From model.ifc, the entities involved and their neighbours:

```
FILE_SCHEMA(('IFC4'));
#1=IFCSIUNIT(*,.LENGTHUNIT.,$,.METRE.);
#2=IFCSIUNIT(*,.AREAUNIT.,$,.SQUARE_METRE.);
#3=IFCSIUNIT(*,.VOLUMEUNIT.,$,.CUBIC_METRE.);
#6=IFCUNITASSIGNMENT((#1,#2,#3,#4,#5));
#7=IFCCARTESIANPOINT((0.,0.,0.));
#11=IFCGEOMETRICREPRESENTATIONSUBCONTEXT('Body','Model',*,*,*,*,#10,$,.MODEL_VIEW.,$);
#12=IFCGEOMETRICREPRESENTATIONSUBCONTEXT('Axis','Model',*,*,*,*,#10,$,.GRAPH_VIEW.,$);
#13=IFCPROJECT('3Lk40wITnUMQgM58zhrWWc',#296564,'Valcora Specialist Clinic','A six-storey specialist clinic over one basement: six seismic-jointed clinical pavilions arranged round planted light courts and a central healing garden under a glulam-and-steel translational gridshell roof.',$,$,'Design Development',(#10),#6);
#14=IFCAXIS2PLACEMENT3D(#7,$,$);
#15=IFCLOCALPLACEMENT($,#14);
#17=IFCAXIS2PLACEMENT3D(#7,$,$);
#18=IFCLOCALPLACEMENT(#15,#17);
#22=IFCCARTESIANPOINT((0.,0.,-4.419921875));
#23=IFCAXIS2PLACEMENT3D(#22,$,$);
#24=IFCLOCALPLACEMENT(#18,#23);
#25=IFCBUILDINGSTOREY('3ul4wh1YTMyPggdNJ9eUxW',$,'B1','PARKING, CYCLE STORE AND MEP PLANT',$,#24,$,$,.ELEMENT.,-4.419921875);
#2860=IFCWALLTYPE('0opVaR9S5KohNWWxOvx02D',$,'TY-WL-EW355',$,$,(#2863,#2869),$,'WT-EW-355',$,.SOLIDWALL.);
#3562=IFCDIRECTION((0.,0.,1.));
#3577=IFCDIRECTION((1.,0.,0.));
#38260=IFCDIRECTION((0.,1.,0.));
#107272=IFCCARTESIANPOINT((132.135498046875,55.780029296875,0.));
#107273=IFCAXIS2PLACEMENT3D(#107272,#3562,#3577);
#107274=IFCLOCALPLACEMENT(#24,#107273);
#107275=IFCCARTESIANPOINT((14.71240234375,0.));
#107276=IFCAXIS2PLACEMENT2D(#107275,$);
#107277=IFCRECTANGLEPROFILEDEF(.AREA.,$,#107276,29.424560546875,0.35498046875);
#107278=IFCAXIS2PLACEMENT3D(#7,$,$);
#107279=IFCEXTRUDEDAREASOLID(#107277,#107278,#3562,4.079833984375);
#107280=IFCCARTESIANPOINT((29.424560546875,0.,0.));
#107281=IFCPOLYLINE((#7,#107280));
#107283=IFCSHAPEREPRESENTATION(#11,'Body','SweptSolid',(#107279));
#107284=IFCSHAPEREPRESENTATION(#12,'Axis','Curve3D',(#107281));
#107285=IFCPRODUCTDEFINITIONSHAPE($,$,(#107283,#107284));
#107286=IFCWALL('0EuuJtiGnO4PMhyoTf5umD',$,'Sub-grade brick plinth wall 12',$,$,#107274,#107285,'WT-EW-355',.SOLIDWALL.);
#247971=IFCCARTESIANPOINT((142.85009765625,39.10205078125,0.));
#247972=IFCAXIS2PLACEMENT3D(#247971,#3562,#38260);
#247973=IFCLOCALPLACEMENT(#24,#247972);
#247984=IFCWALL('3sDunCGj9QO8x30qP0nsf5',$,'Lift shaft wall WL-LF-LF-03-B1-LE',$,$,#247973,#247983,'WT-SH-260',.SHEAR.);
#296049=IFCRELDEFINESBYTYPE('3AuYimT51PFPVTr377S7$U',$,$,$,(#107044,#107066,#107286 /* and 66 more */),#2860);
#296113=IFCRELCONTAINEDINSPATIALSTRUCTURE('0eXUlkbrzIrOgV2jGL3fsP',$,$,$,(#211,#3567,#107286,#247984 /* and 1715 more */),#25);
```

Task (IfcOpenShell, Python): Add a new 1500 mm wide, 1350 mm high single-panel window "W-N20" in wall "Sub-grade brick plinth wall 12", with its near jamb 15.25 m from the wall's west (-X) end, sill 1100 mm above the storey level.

```python
import numpy as np
import ifcopenshell
import ifcopenshell.api.feature
import ifcopenshell.api.geometry
import ifcopenshell.api.root
import ifcopenshell.api.spatial
import ifcopenshell.geom
import ifcopenshell.util.element
import ifcopenshell.util.placement
import ifcopenshell.util.representation
import ifcopenshell.util.shape
import ifcopenshell.util.unit

model = ifcopenshell.open("model.ifc")
unit_scale = ifcopenshell.util.unit.calculate_unit_scale(model)
settings = ifcopenshell.geom.settings()


def volume(element):
    """Net volume in cubic metres, openings subtracted."""
    shape = ifcopenshell.geom.create_shape(settings, element)
    return ifcopenshell.util.shape.get_volume(shape.geometry)


wall = model.by_guid("0EuuJtiGnO4PMhyoTf5umD")
storey = ifcopenshell.util.element.get_container(wall, ifc_class="IfcBuildingStorey")
context = ifcopenshell.util.representation.get_context(model, "Model", "Body", "MODEL_VIEW")
before = volume(wall)

width, height, from_end, sill = 1.5, 1.35, 15.25, 1.1  # metres

# The wall runs along its own X axis, and the end named is its -X end.
wall_shape = ifcopenshell.geom.create_shape(settings, wall)
x, y, z = ifcopenshell.util.shape.get_vertices(wall_shape.geometry).T
start = x.min() + from_end
face, thickness = float(y.min()), float(y.max() - y.min())
wall_matrix = ifcopenshell.util.placement.get_local_placement(wall.ObjectPlacement)
level = ifcopenshell.util.placement.get_local_placement(storey.ObjectPlacement)[2, 3]


def in_wall(x, y):
    """Placement at x, y metres in the wall's axes, at sill height."""
    matrix = wall_matrix.copy()
    matrix[:, 3] = wall_matrix @ np.array([x / unit_scale, y / unit_scale, 0.0, 1.0])
    matrix[2, 3] = level + sill / unit_scale
    return matrix


# Opening: a box that overshoots both wall faces by 50 mm.
opening = ifcopenshell.api.root.create_entity(model, ifc_class="IfcOpeningElement", predefined_type="OPENING")
box = ifcopenshell.api.geometry.add_wall_representation(
    model, context=context, length=width, height=height, thickness=thickness + 0.1
)
ifcopenshell.api.geometry.assign_representation(model, product=opening, representation=box)
ifcopenshell.api.geometry.edit_object_placement(model, product=opening, matrix=in_wall(start, face - 0.05), is_si=False)
ifcopenshell.api.feature.add_feature(model, feature=opening, element=wall)

window = ifcopenshell.api.root.create_entity(model, ifc_class="IfcWindow", name="W-N20", predefined_type="WINDOW")
window.OverallWidth, window.OverallHeight = width / unit_scale, height / unit_scale
window.PartitioningType = "SINGLE_PANEL"
body = ifcopenshell.api.geometry.add_window_representation(
    model,
    context=context,
    overall_width=window.OverallWidth,
    overall_height=window.OverallHeight,
    partition_type="SINGLE_PANEL",
)
ifcopenshell.api.geometry.assign_representation(model, product=window, representation=body)
ifcopenshell.api.spatial.assign_container(model, products=[window], relating_structure=storey)
ifcopenshell.api.feature.add_filling(model, opening=opening, element=window)

# Centre the window in the wall's thickness.
ifcopenshell.api.geometry.edit_object_placement(model, product=window, matrix=in_wall(start, face), is_si=False)
window_shape = ifcopenshell.geom.create_shape(settings, window)
depth = ifcopenshell.util.shape.get_vertices(window_shape.geometry)[:, 1]
offset = face + thickness / 2 - (depth.min() + depth.max()) / 2
ifcopenshell.api.geometry.edit_object_placement(model, product=window, matrix=in_wall(start, offset), is_si=False)

after = volume(wall)

print(f"wall volume {before:.3f} -> {after:.3f} m3")

model.write("model_edited.ifc")
```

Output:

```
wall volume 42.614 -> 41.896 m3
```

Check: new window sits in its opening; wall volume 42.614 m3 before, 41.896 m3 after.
